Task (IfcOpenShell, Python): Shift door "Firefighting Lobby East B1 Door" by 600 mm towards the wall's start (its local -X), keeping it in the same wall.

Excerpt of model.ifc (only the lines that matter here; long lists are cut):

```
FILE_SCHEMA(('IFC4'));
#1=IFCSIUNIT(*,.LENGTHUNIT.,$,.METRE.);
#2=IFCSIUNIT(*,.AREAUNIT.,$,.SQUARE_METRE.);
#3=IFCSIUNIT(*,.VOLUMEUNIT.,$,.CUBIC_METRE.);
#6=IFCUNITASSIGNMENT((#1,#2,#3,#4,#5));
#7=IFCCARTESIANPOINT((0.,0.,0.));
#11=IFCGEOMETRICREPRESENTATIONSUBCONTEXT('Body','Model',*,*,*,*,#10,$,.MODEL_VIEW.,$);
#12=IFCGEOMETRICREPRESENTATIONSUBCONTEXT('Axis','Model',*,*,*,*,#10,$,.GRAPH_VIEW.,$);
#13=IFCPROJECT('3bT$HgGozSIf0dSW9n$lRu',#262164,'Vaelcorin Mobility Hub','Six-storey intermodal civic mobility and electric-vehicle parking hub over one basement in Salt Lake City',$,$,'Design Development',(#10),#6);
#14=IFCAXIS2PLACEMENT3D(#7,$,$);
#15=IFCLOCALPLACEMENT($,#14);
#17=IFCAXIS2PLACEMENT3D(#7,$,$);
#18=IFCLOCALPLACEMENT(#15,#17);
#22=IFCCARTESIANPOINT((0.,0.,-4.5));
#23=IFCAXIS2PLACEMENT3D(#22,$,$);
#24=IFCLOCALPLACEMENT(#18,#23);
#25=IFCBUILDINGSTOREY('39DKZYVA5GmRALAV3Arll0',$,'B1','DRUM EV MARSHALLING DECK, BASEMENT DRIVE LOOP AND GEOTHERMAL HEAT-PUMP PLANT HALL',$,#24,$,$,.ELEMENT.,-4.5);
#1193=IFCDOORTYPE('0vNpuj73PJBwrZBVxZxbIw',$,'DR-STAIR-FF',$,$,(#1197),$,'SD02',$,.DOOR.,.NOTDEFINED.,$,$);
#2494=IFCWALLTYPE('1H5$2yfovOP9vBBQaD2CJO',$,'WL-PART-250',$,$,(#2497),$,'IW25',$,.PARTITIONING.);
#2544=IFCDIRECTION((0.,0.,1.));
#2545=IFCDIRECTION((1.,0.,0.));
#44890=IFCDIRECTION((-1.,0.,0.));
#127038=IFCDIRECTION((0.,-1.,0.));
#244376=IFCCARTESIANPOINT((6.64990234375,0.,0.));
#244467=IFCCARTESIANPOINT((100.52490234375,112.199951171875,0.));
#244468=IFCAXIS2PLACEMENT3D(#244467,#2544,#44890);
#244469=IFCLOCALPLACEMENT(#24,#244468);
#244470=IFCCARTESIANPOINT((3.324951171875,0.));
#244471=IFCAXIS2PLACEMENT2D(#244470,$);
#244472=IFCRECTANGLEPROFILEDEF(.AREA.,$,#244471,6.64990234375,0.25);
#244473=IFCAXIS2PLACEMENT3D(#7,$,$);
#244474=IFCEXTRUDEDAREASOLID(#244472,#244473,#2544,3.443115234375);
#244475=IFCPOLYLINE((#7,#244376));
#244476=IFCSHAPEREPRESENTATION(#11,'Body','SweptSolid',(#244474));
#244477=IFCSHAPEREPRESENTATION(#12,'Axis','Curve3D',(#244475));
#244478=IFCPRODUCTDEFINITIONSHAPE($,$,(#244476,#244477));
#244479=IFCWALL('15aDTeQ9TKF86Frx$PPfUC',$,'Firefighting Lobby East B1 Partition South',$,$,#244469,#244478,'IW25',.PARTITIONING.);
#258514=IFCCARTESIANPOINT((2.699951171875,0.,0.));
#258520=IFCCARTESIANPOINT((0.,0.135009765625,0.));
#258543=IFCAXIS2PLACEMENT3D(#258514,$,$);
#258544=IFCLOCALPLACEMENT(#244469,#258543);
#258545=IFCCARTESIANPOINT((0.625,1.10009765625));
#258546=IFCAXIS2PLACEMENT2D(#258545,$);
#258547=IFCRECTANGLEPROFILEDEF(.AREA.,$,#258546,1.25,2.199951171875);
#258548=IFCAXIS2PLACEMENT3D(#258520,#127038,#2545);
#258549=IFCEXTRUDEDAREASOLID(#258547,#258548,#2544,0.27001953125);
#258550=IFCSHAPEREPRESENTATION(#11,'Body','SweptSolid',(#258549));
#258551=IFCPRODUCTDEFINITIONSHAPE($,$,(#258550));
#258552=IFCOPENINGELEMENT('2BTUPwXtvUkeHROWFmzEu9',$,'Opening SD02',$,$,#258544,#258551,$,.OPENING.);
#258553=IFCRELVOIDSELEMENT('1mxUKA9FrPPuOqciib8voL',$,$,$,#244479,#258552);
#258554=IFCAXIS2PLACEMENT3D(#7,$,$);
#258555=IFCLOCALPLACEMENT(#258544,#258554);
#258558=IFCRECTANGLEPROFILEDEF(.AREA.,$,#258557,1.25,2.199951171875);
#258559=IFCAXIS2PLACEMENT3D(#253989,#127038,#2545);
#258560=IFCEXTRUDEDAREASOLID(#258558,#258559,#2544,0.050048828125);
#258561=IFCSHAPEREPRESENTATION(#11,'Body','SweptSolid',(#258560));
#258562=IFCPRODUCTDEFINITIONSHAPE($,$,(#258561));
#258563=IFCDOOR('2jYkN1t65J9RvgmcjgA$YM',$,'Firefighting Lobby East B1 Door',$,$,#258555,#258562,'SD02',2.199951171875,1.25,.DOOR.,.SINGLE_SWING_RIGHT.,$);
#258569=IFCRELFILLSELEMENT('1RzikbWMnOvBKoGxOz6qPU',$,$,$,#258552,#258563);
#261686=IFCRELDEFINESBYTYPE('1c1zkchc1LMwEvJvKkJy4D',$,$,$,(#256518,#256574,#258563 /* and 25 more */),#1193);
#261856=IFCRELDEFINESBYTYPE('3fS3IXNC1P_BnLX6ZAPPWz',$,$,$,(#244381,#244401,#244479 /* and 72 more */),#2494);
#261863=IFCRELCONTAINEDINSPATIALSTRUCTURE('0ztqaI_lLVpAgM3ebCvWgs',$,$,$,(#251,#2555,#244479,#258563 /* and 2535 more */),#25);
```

```python
import ifcopenshell
import ifcopenshell.api.geometry
import ifcopenshell.util.placement
import ifcopenshell.util.unit

model = ifcopenshell.open("model.ifc")
unit_scale = ifcopenshell.util.unit.calculate_unit_scale(model)

door = model.by_id(258563)
opening = door.FillsVoids[0].RelatingOpeningElement
wall = opening.VoidsElements[0].RelatingBuildingElement

wall_matrix = ifcopenshell.util.placement.get_local_placement(wall.ObjectPlacement)
shift = wall_matrix[:3, 0] * -0.6 / unit_scale
before = ifcopenshell.util.placement.get_local_placement(door.ObjectPlacement)[:3, 3].copy()

# The door is placed relative to its opening, so it follows when the opening moves.
matrix = ifcopenshell.util.placement.get_local_placement(opening.ObjectPlacement)
matrix[:3, 3] += shift
ifcopenshell.api.geometry.edit_object_placement(
    model, product=opening, matrix=matrix, is_si=False, should_transform_children=True
)

after = ifcopenshell.util.placement.get_local_placement(door.ObjectPlacement)[:3, 3]
print("door moved by", (after - before).round(3) + 0.0)

model.write("model_rev.ifc")
```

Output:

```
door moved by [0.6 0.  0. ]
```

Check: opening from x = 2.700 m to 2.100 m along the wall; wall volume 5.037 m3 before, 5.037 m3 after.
